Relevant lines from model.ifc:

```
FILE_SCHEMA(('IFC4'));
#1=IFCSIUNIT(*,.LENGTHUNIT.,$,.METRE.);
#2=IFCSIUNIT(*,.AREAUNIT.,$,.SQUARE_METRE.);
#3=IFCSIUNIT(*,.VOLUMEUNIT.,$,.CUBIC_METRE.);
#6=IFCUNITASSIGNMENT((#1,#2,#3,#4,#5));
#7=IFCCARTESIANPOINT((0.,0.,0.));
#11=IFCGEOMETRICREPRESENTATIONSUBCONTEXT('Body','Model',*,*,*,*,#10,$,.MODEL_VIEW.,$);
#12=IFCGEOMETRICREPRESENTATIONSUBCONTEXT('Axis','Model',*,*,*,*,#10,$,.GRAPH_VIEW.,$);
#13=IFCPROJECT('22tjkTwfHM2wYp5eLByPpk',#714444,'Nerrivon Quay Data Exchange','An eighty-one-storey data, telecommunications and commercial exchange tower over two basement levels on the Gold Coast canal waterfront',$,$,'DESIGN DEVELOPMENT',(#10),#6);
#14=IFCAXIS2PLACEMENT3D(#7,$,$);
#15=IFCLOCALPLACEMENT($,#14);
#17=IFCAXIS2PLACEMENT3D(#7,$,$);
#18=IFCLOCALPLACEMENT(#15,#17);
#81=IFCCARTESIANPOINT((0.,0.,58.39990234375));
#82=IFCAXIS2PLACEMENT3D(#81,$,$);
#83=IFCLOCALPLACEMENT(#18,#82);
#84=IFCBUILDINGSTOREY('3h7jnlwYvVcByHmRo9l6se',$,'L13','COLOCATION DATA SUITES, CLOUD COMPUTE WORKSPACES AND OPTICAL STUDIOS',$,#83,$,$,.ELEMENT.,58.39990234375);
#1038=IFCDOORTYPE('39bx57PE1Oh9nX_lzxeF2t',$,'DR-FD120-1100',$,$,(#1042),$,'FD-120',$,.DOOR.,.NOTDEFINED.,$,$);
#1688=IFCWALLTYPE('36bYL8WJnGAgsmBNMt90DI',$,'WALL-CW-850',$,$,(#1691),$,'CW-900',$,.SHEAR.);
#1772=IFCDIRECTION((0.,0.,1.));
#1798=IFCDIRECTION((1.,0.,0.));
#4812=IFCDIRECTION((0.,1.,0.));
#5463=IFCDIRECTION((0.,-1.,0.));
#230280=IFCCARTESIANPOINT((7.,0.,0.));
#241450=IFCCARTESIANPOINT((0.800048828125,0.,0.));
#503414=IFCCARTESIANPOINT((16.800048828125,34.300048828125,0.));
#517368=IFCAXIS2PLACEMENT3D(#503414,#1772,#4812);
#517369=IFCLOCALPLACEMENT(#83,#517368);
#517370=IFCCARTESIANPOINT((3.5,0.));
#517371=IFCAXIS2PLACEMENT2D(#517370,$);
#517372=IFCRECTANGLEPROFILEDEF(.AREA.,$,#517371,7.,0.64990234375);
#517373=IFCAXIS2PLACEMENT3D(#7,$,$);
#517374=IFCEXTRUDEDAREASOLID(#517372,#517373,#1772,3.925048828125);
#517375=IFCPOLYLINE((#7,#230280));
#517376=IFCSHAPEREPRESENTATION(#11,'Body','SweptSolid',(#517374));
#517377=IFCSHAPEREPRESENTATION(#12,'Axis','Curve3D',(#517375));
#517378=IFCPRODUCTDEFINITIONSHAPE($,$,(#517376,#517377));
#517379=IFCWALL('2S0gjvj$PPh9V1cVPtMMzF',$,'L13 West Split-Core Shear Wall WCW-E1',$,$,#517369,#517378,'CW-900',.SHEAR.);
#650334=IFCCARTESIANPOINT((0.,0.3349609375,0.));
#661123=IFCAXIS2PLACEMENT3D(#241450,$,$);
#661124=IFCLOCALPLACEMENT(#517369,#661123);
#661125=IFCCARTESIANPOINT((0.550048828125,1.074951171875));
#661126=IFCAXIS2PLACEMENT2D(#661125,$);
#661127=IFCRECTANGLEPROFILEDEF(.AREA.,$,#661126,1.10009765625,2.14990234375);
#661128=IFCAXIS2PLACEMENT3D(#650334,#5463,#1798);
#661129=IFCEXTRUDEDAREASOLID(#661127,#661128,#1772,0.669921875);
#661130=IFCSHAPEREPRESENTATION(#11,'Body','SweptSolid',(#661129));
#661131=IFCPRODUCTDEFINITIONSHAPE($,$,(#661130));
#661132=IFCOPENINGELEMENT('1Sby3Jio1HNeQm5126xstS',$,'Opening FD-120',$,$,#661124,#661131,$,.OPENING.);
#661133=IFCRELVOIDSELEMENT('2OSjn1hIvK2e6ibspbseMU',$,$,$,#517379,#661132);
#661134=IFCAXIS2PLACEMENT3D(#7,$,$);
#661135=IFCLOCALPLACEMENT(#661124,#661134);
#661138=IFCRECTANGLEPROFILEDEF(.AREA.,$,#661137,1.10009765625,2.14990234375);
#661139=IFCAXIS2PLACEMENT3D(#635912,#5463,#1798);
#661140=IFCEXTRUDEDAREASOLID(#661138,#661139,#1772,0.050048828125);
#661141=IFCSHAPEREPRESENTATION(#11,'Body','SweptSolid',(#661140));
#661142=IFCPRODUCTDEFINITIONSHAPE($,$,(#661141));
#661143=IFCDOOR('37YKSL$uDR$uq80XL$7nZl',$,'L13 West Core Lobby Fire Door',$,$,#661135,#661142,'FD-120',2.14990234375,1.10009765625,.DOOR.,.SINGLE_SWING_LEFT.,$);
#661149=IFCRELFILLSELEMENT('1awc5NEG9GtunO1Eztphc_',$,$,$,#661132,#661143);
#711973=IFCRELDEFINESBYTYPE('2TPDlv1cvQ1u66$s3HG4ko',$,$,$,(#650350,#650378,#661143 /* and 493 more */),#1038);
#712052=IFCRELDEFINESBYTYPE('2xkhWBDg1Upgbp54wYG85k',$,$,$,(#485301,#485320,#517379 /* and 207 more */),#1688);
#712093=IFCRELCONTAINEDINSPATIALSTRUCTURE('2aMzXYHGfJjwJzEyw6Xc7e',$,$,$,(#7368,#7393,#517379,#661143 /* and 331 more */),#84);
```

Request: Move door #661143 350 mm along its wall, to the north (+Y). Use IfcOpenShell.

```python
import ifcopenshell
import ifcopenshell.api.geometry
import ifcopenshell.util.placement
import ifcopenshell.util.unit

model = ifcopenshell.open("model.ifc")
unit_scale = ifcopenshell.util.unit.calculate_unit_scale(model)

door = model.by_id(661143)
opening = door.FillsVoids[0].RelatingOpeningElement
wall = opening.VoidsElements[0].RelatingBuildingElement

wall_matrix = ifcopenshell.util.placement.get_local_placement(wall.ObjectPlacement)
shift = wall_matrix[:3, 0] * 0.35 / unit_scale
before = ifcopenshell.util.placement.get_local_placement(door.ObjectPlacement)[:3, 3].copy()

# The door is placed relative to its opening, so it follows when the opening moves.
matrix = ifcopenshell.util.placement.get_local_placement(opening.ObjectPlacement)
matrix[:3, 3] += shift
ifcopenshell.api.geometry.edit_object_placement(
    model, product=opening, matrix=matrix, is_si=False, should_transform_children=True
)

after = ifcopenshell.util.placement.get_local_placement(door.ObjectPlacement)[:3, 3]
print("door moved by", (after - before).round(3) + 0.0)

model.write("model_rev.ifc")
```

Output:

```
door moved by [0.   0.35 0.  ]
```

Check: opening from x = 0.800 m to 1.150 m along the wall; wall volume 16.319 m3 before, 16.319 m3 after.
